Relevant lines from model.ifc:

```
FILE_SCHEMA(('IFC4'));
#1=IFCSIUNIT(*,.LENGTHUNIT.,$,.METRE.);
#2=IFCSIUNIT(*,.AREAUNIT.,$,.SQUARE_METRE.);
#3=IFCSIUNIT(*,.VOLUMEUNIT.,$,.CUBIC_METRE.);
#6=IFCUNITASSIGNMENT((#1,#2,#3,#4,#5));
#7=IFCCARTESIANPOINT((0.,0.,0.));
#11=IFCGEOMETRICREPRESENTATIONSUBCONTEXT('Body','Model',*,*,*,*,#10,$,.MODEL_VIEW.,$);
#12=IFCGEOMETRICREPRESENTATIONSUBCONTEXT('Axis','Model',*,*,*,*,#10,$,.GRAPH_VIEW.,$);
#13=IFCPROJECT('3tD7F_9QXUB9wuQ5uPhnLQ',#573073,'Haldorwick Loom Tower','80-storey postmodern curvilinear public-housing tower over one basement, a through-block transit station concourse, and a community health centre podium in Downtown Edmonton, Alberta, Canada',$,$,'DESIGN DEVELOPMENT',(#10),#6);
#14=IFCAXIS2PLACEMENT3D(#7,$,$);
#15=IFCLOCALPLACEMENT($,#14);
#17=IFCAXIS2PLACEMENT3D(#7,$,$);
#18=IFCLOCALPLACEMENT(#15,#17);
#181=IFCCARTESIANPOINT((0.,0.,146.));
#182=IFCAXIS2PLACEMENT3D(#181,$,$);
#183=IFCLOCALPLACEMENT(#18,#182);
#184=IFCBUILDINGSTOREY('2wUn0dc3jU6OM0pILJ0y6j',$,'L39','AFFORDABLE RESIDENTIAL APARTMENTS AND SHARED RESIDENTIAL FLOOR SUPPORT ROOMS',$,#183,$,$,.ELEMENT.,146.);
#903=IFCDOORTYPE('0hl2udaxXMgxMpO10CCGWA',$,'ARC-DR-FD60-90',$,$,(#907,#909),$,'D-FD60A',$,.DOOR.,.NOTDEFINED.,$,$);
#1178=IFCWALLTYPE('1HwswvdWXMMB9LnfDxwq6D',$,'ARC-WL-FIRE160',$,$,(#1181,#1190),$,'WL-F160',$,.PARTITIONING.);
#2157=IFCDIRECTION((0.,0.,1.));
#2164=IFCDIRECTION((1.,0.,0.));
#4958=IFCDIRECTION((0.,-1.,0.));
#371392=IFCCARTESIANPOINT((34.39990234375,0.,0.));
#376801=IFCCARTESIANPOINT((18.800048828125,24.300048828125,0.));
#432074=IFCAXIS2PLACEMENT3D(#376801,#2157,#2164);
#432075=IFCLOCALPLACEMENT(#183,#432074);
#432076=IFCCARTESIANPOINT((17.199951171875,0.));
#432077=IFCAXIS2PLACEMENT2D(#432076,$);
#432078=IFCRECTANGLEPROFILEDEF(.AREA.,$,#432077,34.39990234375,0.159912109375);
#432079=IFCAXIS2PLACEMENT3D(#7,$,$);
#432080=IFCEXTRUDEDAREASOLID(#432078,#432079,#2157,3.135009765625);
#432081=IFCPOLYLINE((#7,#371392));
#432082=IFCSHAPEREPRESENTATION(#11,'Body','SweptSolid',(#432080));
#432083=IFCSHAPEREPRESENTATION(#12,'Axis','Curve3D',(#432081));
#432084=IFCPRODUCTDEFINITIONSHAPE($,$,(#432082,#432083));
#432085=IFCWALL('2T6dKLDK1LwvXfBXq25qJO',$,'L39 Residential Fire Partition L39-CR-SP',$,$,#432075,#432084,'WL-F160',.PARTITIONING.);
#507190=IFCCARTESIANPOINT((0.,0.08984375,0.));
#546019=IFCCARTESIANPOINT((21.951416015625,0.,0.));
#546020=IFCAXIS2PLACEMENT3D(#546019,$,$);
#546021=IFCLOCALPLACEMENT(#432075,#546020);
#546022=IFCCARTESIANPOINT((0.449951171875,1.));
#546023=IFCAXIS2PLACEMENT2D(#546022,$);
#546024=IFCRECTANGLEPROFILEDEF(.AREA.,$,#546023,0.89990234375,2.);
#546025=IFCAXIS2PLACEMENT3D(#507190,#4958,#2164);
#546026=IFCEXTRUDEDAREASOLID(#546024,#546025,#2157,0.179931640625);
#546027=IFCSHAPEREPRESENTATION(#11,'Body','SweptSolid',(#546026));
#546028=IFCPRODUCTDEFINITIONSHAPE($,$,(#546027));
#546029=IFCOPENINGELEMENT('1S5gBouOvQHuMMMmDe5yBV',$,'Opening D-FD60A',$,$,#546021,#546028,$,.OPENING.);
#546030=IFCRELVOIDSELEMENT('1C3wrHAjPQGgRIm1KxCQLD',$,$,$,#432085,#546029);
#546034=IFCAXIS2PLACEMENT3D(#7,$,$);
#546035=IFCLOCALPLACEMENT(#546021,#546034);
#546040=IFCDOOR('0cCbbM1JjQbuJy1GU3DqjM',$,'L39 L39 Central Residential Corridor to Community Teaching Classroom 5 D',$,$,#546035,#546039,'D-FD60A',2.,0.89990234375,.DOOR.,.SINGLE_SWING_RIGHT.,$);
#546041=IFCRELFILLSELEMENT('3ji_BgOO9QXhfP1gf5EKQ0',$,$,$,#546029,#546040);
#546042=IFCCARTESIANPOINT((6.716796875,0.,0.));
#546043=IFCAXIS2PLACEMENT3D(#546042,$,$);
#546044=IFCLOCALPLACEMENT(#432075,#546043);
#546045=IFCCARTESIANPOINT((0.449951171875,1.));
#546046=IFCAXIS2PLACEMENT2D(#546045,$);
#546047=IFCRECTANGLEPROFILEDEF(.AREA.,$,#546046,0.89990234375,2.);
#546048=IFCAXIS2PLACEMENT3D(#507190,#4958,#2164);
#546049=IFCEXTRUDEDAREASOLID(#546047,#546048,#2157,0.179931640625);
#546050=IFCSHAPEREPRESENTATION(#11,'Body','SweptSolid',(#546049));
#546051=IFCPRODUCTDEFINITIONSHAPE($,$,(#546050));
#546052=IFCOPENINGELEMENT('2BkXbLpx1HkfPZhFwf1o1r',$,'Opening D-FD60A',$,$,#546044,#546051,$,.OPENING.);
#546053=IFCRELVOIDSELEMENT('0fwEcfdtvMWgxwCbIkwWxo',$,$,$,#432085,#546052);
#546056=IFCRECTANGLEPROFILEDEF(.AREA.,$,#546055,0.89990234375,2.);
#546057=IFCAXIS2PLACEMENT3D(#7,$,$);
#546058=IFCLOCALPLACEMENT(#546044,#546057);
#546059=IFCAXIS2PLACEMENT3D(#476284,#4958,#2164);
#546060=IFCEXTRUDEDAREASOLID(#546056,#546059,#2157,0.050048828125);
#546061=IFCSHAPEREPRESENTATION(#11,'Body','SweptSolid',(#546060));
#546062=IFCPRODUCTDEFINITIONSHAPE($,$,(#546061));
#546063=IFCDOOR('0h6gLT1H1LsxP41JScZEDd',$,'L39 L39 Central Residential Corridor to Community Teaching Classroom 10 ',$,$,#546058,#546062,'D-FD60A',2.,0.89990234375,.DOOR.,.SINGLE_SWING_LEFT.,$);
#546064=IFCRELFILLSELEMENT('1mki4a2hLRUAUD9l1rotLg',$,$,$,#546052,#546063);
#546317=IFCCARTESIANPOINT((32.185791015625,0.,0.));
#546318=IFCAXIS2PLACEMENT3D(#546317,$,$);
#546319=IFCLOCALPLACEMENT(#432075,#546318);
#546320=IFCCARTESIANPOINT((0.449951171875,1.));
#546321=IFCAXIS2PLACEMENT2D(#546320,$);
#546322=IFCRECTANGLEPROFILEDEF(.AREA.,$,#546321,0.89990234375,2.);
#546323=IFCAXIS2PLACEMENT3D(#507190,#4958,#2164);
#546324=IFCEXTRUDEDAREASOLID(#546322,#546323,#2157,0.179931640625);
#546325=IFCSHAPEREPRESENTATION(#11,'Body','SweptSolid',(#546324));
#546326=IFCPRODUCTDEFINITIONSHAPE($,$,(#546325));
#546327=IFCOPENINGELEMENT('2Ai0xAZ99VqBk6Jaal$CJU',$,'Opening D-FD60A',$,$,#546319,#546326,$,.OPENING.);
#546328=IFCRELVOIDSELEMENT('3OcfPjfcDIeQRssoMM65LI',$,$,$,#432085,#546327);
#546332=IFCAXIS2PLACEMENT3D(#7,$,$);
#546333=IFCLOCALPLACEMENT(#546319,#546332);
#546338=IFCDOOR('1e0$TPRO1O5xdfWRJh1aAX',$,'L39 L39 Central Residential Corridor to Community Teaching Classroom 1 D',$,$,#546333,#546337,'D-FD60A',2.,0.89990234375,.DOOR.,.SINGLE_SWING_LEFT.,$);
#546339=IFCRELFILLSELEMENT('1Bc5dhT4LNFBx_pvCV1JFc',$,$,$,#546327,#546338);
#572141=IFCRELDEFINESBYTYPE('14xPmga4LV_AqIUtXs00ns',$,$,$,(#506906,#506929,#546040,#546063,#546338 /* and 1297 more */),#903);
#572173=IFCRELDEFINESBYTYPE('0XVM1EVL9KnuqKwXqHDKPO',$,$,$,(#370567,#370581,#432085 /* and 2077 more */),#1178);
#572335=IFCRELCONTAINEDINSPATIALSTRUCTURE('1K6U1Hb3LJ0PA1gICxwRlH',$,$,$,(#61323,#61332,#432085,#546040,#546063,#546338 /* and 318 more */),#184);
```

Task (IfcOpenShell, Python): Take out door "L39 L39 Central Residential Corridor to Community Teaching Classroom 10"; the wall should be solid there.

```python
import ifcopenshell
import ifcopenshell.api.feature
import ifcopenshell.api.root
import ifcopenshell.geom
import ifcopenshell.util.shape

model = ifcopenshell.open("model.ifc")
settings = ifcopenshell.geom.settings()


def volume(element):
    """Net volume in cubic metres, openings subtracted."""
    shape = ifcopenshell.geom.create_shape(settings, element)
    return ifcopenshell.util.shape.get_volume(shape.geometry)


door = model.by_guid("0h6gLT1H1LsxP41JScZEDd")
opening = door.FillsVoids[0].RelatingOpeningElement
wall = opening.VoidsElements[0].RelatingBuildingElement
before = volume(wall)

ifcopenshell.api.root.remove_product(model, product=door)
ifcopenshell.api.feature.remove_feature(model, feature=opening)

after = volume(wall)

print(f"wall volume {before:.3f} -> {after:.3f} m3")

model.write("model_updated.ifc")
```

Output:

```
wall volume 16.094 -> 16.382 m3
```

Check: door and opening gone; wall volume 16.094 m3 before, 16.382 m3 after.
